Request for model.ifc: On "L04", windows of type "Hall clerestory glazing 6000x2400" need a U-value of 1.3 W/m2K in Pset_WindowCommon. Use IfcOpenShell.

First a look at what the model holds.

```python
import ifcopenshell
import ifcopenshell.util.element

model = ifcopenshell.open("model.ifc")
print(model.schema)
storey = next(s for s in model.by_type("IfcBuildingStorey") if s.Name == "L04")
windows = [e for e in ifcopenshell.util.element.get_decomposition(storey) if e.is_a("IfcWindow")]
seen = {}
for e in windows:
    element_type = ifcopenshell.util.element.get_type(e)
    key = (element_type.Name if element_type != e and element_type else None, ifcopenshell.util.element.get_pset(e, "Pset_WindowCommon", "ThermalTransmittance"))
    seen[key] = seen.get(key, 0) + 1
for (name, value), count in sorted(seen.items(), key=str):
    print(count, "x", name, "|", value)
```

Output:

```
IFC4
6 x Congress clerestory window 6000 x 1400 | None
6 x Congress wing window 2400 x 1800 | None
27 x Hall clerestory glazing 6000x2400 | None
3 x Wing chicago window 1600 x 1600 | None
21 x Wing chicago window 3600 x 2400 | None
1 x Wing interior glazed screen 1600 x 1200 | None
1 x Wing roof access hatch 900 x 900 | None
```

```python
import ifcopenshell
import ifcopenshell.api.pset
import ifcopenshell.util.element

model = ifcopenshell.open("model.ifc")

storey = next(s for s in model.by_type("IfcBuildingStorey") if s.Name == "L04")
windows = [e for e in ifcopenshell.util.element.get_decomposition(storey) if e.is_a("IfcWindow")]

count = 0
for e in windows:
    element_type = ifcopenshell.util.element.get_type(e)
    if element_type in (None, e) or element_type.Name != "Hall clerestory glazing 6000x2400":
        continue
    # add_pset returns the element's existing set when there is one.
    pset = ifcopenshell.api.pset.add_pset(model, product=e, name="Pset_WindowCommon")
    ifcopenshell.api.pset.edit_pset(model, pset=pset, properties={"ThermalTransmittance": 1.3})
    count += 1

print(count, "windows updated")

model.write("model-out.ifc")
```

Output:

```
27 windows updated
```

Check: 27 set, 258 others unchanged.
